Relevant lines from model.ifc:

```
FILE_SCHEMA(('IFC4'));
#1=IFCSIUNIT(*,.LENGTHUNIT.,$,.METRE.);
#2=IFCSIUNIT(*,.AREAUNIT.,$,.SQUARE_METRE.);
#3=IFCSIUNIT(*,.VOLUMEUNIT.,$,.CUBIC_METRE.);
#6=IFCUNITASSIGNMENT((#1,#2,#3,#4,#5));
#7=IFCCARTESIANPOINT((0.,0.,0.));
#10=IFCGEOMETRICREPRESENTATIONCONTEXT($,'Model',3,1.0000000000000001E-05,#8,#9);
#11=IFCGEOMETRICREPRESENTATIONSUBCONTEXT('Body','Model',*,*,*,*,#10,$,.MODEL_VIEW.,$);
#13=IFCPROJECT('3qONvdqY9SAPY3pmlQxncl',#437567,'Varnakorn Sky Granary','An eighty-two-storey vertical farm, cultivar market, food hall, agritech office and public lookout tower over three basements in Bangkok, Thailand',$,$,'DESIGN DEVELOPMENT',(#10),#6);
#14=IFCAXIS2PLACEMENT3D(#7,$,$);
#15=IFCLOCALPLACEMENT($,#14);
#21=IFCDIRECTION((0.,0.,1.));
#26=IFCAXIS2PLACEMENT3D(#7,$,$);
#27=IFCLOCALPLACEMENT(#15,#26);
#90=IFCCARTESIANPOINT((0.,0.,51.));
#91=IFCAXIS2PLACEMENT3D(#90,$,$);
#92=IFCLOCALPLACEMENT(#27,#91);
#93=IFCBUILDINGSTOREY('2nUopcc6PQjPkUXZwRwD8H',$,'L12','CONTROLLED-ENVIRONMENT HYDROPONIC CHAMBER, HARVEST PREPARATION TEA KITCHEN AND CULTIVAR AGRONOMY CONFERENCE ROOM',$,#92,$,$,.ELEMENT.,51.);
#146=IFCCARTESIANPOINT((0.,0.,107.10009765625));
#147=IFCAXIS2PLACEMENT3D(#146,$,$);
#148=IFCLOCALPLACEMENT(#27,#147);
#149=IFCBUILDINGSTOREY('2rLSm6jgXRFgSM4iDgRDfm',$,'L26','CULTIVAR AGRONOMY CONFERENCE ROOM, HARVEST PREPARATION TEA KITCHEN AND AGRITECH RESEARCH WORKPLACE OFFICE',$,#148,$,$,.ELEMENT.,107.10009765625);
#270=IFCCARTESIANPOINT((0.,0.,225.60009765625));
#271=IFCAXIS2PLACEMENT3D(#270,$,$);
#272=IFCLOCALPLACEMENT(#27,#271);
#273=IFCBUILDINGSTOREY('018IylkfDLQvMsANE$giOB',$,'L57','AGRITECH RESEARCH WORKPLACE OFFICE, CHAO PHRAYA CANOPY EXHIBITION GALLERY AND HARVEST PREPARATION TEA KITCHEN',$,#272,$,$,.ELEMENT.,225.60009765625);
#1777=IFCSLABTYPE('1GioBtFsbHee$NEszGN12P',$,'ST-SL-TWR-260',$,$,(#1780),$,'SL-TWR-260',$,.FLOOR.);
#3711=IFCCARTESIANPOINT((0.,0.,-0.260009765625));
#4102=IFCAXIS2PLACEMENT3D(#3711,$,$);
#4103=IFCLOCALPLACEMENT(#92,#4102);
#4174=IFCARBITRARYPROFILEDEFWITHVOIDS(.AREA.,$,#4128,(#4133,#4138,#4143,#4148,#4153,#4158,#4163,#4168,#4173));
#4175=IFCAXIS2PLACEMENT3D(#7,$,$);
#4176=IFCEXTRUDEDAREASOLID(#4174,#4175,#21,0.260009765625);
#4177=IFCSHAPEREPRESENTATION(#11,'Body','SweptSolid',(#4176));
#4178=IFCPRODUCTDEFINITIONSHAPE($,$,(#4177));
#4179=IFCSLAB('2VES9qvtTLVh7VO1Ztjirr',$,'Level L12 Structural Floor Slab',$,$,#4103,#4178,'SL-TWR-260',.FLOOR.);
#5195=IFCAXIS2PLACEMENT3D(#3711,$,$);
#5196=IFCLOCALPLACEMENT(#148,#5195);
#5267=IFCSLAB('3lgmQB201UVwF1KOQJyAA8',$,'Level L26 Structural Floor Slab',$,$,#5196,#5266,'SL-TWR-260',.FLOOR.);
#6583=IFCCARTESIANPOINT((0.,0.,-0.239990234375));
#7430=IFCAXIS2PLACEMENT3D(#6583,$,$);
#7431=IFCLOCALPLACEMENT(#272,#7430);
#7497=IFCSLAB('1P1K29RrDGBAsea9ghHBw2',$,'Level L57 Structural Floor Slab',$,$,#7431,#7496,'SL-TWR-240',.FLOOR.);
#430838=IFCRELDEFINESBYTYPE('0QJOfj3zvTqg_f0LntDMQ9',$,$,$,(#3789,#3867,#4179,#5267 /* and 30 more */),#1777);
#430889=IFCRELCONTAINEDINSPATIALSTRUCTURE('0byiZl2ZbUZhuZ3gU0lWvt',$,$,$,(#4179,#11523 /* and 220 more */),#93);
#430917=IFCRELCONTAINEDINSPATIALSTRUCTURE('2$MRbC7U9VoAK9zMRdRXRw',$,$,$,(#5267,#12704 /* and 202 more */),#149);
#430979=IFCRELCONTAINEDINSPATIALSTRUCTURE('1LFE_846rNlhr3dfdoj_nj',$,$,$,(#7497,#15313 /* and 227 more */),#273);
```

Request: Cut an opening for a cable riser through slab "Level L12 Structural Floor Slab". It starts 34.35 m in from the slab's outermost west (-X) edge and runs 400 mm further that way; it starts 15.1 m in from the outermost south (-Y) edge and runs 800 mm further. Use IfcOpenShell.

```python
import numpy as np
import ifcopenshell
import ifcopenshell.api.feature
import ifcopenshell.api.geometry
import ifcopenshell.api.root
import ifcopenshell.geom
import ifcopenshell.util.placement
import ifcopenshell.util.representation
import ifcopenshell.util.shape
import ifcopenshell.util.unit

model = ifcopenshell.open("model.ifc")
unit_scale = ifcopenshell.util.unit.calculate_unit_scale(model)
settings = ifcopenshell.geom.settings()


def volume(element):
    """Net volume in cubic metres, openings subtracted."""
    shape = ifcopenshell.geom.create_shape(settings, element)
    return ifcopenshell.util.shape.get_volume(shape.geometry)


slab = model.by_guid("2VES9qvtTLVh7VO1Ztjirr")
before = volume(slab)

# Extent in the slab's own axes, in metres. The edges named are its -X and -Y sides.
slab_shape = ifcopenshell.geom.create_shape(settings, slab)
vertices = ifcopenshell.util.shape.get_vertices(slab_shape.geometry)
x_min, y_min, bottom = vertices.min(axis=0)
top = vertices[:, 2].max()

opening = ifcopenshell.api.root.create_entity(model, ifc_class="IfcOpeningElement", name="Cable riser opening", predefined_type="OPENING")
context = ifcopenshell.util.representation.get_context(model, "Model", "Body", "MODEL_VIEW")
width, depth = 0.4, 0.8
outline = [(0.0, 0.0), (width, 0.0), (width, depth), (0.0, depth), (0.0, 0.0)]
# Overshoot both faces by 50 mm so the cut is clean.
shape = ifcopenshell.api.geometry.add_slab_representation(
    model, context=context, depth=top - bottom + 0.1, polyline=outline
)
ifcopenshell.api.geometry.assign_representation(model, product=opening, representation=shape)

matrix = ifcopenshell.util.placement.get_local_placement(slab.ObjectPlacement)
matrix[:, 3] = matrix @ np.append(np.array([x_min + 34.35, y_min + 15.1, bottom - 0.05]) / unit_scale, 1.0)
ifcopenshell.api.geometry.edit_object_placement(model, product=opening, matrix=matrix, is_si=False)
ifcopenshell.api.feature.add_feature(model, feature=opening, element=slab)

after = volume(slab)

print(f"slab volume {before:.3f} -> {after:.3f} m3")

model.write("model_edited.ifc")
```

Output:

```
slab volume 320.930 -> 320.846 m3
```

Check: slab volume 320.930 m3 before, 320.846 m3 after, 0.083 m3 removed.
